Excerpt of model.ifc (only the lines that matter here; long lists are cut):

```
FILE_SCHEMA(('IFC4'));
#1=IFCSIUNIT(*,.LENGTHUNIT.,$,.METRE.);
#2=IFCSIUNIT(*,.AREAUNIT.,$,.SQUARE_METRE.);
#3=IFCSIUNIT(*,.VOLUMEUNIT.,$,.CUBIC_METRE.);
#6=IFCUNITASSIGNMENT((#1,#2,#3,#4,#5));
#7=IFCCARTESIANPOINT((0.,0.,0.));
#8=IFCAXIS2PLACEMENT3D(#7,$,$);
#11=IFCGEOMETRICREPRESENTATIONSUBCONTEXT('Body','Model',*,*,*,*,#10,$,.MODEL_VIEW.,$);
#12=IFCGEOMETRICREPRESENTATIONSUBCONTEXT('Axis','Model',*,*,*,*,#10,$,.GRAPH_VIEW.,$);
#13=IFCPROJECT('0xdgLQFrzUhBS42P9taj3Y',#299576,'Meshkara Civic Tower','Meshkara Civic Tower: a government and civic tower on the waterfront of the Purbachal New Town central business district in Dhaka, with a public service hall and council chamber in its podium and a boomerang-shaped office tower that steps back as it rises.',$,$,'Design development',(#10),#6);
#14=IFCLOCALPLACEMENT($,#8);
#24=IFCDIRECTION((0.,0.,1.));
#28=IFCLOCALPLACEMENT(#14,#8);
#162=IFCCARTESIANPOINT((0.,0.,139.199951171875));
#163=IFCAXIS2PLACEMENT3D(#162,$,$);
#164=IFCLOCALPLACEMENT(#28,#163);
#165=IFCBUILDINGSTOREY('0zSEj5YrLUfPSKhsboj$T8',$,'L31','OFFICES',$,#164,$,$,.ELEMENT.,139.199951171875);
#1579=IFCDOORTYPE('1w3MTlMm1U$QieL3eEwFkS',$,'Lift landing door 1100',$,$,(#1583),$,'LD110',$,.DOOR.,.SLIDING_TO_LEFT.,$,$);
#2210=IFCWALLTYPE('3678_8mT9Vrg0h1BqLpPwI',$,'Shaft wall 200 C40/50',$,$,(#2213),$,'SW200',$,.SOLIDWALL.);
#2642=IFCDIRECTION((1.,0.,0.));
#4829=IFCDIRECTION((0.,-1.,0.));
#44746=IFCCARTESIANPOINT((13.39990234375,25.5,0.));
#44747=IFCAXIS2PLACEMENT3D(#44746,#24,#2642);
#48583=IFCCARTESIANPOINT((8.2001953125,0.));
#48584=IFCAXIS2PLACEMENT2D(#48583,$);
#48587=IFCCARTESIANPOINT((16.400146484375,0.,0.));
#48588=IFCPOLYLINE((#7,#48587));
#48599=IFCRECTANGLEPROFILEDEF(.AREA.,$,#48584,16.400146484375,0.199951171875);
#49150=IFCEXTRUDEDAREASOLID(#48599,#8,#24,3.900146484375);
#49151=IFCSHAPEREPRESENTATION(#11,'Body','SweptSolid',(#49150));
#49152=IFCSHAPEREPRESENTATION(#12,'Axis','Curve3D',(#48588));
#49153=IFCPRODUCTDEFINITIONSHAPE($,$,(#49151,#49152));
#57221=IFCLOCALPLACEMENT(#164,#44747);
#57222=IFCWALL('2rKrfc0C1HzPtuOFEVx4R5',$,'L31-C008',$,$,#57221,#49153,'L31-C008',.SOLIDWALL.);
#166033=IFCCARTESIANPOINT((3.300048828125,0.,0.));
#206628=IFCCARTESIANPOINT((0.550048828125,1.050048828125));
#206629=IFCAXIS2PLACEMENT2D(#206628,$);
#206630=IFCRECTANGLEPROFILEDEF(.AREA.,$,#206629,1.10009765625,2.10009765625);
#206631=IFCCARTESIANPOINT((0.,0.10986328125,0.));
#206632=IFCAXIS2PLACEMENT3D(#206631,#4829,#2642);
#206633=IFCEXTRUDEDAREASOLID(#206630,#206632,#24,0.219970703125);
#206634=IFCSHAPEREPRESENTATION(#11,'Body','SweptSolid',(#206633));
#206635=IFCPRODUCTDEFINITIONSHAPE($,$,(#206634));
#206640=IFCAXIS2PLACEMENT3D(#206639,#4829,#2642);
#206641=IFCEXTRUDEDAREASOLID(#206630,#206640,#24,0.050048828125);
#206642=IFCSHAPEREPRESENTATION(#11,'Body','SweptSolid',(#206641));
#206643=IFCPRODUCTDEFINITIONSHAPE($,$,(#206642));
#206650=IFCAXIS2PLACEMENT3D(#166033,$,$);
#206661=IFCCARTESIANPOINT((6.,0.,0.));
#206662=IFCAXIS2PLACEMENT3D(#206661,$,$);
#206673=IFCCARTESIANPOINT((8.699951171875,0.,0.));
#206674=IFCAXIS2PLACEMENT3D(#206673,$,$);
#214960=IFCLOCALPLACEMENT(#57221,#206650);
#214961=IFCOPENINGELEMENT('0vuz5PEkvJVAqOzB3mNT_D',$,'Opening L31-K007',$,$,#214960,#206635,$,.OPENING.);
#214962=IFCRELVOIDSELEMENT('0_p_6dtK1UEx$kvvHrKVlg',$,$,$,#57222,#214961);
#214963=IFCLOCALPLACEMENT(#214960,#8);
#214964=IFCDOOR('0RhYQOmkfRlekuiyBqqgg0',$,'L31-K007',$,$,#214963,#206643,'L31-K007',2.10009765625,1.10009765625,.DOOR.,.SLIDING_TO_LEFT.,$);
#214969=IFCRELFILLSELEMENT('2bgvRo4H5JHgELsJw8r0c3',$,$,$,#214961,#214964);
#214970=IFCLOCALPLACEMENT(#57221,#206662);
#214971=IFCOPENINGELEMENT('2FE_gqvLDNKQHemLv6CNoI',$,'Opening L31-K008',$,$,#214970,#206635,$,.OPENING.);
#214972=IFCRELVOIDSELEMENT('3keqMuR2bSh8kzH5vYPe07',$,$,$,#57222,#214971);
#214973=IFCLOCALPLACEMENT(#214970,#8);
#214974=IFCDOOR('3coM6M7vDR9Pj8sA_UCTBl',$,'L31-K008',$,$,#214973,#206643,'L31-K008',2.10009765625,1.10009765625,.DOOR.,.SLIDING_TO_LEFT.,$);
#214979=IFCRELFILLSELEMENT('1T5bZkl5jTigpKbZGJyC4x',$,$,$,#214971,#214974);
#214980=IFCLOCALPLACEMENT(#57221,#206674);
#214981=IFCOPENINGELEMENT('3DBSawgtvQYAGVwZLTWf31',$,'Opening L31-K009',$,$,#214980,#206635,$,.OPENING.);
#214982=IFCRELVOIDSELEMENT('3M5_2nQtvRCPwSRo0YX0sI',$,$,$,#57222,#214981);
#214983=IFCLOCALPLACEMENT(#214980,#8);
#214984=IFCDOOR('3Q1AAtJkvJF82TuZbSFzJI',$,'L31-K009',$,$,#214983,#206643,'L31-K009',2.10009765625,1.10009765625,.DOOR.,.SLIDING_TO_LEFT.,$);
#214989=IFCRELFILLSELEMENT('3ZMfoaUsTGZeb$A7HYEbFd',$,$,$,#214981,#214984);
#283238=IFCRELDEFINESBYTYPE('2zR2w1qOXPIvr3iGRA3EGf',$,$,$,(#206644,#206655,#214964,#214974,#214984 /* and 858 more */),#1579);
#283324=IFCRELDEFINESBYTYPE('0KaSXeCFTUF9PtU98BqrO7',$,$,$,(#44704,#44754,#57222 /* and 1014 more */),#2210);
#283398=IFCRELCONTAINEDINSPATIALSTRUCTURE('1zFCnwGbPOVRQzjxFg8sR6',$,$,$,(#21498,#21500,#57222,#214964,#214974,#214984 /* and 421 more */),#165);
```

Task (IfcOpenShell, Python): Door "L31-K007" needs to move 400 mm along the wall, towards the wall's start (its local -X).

```python
import ifcopenshell
import ifcopenshell.api.geometry
import ifcopenshell.util.placement

model = ifcopenshell.open("model.ifc")

door = model.by_guid("0RhYQOmkfRlekuiyBqqgg0")
opening = door.FillsVoids[0].RelatingOpeningElement
wall = opening.VoidsElements[0].RelatingBuildingElement

wall_matrix = ifcopenshell.util.placement.get_local_placement(wall.ObjectPlacement)
shift = wall_matrix[:3, 0] * -0.4
before = ifcopenshell.util.placement.get_local_placement(door.ObjectPlacement)[:3, 3].copy()

# The door is placed relative to its opening, so it follows when the opening moves.
matrix = ifcopenshell.util.placement.get_local_placement(opening.ObjectPlacement)
matrix[:3, 3] += shift
ifcopenshell.api.geometry.edit_object_placement(
    model, product=opening, matrix=matrix, is_si=False, should_transform_children=True
)

after = ifcopenshell.util.placement.get_local_placement(door.ObjectPlacement)[:3, 3]
print("door moved by", (after - before).round(3) + 0.0)

model.write("model_edited.ifc")
```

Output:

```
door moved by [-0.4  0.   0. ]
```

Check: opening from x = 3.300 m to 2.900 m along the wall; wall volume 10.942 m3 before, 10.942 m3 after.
